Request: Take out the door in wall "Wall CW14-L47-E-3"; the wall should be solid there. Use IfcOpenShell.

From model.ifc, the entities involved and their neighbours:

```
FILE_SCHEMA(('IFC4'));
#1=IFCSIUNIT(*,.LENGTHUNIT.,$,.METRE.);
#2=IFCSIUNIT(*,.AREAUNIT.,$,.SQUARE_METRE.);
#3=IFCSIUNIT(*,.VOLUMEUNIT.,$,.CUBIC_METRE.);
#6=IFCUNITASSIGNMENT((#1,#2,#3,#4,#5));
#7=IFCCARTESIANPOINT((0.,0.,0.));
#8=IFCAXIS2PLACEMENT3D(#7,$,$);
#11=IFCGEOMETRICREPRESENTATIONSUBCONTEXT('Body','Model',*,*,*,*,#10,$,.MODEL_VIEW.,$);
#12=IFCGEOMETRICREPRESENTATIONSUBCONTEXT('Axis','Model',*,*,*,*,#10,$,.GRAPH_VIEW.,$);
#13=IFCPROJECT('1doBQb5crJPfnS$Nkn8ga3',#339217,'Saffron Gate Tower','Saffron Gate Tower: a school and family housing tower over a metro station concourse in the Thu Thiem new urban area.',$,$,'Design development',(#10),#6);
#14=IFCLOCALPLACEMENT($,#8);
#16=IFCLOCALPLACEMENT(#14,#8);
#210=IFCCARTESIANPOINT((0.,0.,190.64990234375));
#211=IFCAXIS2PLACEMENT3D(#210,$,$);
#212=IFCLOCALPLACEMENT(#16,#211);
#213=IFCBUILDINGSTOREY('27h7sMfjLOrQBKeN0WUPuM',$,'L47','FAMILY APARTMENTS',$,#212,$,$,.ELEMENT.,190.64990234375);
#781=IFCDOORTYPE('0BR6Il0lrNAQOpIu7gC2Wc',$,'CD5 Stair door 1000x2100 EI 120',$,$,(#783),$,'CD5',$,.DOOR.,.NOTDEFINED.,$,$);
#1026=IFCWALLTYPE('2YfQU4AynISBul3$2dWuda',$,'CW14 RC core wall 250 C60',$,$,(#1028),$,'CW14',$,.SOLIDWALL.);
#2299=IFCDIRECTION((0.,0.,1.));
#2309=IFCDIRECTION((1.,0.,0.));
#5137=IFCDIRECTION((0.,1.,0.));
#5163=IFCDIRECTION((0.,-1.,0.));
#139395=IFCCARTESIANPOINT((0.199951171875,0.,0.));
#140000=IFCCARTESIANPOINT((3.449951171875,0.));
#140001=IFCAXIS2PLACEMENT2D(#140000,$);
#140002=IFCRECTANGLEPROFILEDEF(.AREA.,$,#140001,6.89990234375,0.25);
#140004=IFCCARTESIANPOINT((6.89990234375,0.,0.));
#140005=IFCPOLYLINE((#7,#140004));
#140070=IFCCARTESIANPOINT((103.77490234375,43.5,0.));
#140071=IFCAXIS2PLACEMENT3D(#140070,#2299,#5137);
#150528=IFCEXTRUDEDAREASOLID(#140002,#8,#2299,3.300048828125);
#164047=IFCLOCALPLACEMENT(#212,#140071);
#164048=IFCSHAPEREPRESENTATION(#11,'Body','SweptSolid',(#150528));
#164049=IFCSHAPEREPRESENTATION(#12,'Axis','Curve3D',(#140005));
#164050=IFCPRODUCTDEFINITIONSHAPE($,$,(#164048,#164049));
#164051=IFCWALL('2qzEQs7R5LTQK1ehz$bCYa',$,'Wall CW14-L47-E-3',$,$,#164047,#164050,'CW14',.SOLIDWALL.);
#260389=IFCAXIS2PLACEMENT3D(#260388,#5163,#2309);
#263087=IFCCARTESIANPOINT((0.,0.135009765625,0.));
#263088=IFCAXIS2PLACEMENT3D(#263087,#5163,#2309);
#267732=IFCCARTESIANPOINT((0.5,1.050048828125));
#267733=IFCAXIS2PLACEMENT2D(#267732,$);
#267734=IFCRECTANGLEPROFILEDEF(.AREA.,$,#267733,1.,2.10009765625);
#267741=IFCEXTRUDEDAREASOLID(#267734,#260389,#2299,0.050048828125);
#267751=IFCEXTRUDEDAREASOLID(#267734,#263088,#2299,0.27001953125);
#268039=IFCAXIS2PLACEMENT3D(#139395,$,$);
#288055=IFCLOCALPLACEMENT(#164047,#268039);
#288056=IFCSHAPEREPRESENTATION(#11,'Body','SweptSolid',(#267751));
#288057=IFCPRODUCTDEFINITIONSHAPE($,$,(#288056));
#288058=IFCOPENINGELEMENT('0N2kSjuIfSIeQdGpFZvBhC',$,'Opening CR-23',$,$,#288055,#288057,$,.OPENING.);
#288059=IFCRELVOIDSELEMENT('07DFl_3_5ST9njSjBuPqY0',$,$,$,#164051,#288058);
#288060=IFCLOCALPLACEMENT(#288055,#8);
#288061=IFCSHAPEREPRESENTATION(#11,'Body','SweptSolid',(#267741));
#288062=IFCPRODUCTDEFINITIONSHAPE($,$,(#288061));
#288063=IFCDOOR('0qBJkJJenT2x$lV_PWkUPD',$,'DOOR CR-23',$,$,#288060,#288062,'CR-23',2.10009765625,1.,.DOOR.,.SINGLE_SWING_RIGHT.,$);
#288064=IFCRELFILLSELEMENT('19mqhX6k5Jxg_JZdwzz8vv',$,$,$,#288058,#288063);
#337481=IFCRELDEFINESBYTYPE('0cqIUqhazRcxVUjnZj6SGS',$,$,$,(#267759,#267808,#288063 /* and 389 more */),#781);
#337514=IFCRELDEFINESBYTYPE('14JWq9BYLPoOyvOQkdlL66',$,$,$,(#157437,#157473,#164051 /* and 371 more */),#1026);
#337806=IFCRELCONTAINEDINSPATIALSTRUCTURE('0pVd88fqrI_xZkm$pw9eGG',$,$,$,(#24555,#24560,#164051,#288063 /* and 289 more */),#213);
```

```python
import ifcopenshell
import ifcopenshell.api.feature
import ifcopenshell.api.root
import ifcopenshell.geom
import ifcopenshell.util.shape

model = ifcopenshell.open("model.ifc")
settings = ifcopenshell.geom.settings()


def volume(element):
    """Net volume in cubic metres, openings subtracted."""
    shape = ifcopenshell.geom.create_shape(settings, element)
    return ifcopenshell.util.shape.get_volume(shape.geometry)


door = model.by_guid("0qBJkJJenT2x$lV_PWkUPD")
opening = door.FillsVoids[0].RelatingOpeningElement
wall = opening.VoidsElements[0].RelatingBuildingElement
before = volume(wall)

ifcopenshell.api.root.remove_product(model, product=door)
ifcopenshell.api.feature.remove_feature(model, feature=opening)

after = volume(wall)

print(f"wall volume {before:.3f} -> {after:.3f} m3")

model.write("model_updated.ifc")
```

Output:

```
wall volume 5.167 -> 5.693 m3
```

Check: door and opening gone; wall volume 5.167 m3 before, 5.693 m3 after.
